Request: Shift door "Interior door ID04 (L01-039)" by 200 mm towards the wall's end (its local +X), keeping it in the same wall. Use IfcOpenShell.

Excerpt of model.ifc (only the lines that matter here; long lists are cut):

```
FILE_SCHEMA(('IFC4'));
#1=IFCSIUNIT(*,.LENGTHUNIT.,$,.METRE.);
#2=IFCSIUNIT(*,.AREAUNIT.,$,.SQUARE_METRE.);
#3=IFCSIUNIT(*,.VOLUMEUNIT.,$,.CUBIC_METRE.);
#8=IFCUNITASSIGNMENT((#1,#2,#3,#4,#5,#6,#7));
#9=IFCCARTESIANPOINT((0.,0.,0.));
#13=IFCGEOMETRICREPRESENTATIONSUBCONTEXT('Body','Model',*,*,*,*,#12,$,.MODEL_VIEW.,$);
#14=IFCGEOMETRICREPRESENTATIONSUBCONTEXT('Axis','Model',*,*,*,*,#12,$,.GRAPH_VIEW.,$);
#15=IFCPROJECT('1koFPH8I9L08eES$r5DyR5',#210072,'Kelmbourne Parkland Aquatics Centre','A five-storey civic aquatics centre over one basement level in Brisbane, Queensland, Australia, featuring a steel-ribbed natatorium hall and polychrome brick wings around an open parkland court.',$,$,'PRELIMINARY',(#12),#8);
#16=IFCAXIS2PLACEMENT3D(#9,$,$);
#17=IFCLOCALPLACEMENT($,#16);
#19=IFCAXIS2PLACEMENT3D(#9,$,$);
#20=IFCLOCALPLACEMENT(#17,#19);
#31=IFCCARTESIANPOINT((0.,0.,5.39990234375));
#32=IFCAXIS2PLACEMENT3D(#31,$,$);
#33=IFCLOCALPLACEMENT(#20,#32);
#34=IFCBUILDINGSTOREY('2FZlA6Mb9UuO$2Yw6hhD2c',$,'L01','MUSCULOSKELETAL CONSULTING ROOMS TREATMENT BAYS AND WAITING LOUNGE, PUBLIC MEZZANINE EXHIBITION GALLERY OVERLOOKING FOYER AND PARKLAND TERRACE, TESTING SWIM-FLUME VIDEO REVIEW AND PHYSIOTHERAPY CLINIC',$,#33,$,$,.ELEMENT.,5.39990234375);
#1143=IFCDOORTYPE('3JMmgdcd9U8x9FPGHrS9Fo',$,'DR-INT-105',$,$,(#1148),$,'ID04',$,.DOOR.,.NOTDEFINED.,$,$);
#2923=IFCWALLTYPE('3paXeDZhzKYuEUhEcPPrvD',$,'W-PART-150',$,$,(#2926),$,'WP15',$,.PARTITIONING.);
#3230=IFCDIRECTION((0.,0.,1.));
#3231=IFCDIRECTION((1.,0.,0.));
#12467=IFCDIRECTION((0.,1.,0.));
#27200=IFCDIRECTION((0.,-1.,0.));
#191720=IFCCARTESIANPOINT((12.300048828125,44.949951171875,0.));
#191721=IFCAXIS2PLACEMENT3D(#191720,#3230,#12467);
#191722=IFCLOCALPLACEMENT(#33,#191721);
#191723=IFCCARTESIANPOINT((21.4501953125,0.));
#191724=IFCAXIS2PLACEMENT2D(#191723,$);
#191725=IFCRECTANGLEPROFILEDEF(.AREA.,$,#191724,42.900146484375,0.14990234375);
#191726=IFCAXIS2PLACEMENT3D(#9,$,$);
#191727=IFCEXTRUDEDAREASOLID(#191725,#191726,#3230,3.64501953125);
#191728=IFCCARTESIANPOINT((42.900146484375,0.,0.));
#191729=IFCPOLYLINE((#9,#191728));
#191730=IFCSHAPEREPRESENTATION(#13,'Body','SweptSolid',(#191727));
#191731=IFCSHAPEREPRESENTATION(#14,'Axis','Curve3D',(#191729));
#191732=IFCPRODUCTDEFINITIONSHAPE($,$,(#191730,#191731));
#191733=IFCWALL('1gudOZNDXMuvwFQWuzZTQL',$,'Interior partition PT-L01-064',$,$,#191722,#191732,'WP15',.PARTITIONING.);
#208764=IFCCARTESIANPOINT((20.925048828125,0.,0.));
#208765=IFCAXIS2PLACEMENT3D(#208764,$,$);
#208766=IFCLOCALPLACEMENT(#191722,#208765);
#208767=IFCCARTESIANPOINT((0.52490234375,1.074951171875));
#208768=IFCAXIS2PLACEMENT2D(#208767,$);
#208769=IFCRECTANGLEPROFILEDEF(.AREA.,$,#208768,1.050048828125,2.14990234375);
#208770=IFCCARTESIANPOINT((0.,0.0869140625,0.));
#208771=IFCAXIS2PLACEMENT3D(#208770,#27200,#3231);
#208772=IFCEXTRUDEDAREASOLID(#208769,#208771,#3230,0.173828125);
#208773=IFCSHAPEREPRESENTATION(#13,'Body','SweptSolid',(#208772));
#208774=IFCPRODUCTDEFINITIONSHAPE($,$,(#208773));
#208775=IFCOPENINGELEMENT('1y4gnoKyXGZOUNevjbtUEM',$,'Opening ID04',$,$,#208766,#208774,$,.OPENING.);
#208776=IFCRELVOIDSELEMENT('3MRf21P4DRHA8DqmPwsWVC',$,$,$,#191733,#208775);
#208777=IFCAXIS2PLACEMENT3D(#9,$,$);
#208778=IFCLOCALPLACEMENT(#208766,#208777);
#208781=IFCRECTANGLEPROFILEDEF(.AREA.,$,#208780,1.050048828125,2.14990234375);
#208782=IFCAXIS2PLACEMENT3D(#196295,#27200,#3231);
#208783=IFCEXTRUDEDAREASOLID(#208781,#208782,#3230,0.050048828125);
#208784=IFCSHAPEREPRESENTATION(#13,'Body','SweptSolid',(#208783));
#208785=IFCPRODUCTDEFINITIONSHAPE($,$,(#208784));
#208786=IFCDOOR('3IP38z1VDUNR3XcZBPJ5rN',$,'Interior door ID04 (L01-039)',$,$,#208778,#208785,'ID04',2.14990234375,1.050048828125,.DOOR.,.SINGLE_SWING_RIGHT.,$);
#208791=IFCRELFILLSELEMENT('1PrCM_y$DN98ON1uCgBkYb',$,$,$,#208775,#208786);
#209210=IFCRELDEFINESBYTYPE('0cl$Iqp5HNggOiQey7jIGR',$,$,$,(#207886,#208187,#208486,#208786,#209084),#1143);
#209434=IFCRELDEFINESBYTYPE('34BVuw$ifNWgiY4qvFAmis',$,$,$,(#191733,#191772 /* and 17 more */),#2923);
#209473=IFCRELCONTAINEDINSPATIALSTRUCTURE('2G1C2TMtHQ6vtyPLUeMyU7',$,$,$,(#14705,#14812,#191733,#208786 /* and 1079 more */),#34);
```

```python
import ifcopenshell
import ifcopenshell.api.geometry
import ifcopenshell.util.placement

model = ifcopenshell.open("model.ifc")

door = model.by_guid("3IP38z1VDUNR3XcZBPJ5rN")
opening = door.FillsVoids[0].RelatingOpeningElement
wall = opening.VoidsElements[0].RelatingBuildingElement

wall_matrix = ifcopenshell.util.placement.get_local_placement(wall.ObjectPlacement)
shift = wall_matrix[:3, 0] * 0.2
before = ifcopenshell.util.placement.get_local_placement(door.ObjectPlacement)[:3, 3].copy()

# The door is placed relative to its opening, so it follows when the opening moves.
matrix = ifcopenshell.util.placement.get_local_placement(opening.ObjectPlacement)
matrix[:3, 3] += shift
ifcopenshell.api.geometry.edit_object_placement(
    model, product=opening, matrix=matrix, is_si=False, should_transform_children=True
)

after = ifcopenshell.util.placement.get_local_placement(door.ObjectPlacement)[:3, 3]
print("door moved by", (after - before).round(3) + 0.0)

model.write("model_rev.ifc")
```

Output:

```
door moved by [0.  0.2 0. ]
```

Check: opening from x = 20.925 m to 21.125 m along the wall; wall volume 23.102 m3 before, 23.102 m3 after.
